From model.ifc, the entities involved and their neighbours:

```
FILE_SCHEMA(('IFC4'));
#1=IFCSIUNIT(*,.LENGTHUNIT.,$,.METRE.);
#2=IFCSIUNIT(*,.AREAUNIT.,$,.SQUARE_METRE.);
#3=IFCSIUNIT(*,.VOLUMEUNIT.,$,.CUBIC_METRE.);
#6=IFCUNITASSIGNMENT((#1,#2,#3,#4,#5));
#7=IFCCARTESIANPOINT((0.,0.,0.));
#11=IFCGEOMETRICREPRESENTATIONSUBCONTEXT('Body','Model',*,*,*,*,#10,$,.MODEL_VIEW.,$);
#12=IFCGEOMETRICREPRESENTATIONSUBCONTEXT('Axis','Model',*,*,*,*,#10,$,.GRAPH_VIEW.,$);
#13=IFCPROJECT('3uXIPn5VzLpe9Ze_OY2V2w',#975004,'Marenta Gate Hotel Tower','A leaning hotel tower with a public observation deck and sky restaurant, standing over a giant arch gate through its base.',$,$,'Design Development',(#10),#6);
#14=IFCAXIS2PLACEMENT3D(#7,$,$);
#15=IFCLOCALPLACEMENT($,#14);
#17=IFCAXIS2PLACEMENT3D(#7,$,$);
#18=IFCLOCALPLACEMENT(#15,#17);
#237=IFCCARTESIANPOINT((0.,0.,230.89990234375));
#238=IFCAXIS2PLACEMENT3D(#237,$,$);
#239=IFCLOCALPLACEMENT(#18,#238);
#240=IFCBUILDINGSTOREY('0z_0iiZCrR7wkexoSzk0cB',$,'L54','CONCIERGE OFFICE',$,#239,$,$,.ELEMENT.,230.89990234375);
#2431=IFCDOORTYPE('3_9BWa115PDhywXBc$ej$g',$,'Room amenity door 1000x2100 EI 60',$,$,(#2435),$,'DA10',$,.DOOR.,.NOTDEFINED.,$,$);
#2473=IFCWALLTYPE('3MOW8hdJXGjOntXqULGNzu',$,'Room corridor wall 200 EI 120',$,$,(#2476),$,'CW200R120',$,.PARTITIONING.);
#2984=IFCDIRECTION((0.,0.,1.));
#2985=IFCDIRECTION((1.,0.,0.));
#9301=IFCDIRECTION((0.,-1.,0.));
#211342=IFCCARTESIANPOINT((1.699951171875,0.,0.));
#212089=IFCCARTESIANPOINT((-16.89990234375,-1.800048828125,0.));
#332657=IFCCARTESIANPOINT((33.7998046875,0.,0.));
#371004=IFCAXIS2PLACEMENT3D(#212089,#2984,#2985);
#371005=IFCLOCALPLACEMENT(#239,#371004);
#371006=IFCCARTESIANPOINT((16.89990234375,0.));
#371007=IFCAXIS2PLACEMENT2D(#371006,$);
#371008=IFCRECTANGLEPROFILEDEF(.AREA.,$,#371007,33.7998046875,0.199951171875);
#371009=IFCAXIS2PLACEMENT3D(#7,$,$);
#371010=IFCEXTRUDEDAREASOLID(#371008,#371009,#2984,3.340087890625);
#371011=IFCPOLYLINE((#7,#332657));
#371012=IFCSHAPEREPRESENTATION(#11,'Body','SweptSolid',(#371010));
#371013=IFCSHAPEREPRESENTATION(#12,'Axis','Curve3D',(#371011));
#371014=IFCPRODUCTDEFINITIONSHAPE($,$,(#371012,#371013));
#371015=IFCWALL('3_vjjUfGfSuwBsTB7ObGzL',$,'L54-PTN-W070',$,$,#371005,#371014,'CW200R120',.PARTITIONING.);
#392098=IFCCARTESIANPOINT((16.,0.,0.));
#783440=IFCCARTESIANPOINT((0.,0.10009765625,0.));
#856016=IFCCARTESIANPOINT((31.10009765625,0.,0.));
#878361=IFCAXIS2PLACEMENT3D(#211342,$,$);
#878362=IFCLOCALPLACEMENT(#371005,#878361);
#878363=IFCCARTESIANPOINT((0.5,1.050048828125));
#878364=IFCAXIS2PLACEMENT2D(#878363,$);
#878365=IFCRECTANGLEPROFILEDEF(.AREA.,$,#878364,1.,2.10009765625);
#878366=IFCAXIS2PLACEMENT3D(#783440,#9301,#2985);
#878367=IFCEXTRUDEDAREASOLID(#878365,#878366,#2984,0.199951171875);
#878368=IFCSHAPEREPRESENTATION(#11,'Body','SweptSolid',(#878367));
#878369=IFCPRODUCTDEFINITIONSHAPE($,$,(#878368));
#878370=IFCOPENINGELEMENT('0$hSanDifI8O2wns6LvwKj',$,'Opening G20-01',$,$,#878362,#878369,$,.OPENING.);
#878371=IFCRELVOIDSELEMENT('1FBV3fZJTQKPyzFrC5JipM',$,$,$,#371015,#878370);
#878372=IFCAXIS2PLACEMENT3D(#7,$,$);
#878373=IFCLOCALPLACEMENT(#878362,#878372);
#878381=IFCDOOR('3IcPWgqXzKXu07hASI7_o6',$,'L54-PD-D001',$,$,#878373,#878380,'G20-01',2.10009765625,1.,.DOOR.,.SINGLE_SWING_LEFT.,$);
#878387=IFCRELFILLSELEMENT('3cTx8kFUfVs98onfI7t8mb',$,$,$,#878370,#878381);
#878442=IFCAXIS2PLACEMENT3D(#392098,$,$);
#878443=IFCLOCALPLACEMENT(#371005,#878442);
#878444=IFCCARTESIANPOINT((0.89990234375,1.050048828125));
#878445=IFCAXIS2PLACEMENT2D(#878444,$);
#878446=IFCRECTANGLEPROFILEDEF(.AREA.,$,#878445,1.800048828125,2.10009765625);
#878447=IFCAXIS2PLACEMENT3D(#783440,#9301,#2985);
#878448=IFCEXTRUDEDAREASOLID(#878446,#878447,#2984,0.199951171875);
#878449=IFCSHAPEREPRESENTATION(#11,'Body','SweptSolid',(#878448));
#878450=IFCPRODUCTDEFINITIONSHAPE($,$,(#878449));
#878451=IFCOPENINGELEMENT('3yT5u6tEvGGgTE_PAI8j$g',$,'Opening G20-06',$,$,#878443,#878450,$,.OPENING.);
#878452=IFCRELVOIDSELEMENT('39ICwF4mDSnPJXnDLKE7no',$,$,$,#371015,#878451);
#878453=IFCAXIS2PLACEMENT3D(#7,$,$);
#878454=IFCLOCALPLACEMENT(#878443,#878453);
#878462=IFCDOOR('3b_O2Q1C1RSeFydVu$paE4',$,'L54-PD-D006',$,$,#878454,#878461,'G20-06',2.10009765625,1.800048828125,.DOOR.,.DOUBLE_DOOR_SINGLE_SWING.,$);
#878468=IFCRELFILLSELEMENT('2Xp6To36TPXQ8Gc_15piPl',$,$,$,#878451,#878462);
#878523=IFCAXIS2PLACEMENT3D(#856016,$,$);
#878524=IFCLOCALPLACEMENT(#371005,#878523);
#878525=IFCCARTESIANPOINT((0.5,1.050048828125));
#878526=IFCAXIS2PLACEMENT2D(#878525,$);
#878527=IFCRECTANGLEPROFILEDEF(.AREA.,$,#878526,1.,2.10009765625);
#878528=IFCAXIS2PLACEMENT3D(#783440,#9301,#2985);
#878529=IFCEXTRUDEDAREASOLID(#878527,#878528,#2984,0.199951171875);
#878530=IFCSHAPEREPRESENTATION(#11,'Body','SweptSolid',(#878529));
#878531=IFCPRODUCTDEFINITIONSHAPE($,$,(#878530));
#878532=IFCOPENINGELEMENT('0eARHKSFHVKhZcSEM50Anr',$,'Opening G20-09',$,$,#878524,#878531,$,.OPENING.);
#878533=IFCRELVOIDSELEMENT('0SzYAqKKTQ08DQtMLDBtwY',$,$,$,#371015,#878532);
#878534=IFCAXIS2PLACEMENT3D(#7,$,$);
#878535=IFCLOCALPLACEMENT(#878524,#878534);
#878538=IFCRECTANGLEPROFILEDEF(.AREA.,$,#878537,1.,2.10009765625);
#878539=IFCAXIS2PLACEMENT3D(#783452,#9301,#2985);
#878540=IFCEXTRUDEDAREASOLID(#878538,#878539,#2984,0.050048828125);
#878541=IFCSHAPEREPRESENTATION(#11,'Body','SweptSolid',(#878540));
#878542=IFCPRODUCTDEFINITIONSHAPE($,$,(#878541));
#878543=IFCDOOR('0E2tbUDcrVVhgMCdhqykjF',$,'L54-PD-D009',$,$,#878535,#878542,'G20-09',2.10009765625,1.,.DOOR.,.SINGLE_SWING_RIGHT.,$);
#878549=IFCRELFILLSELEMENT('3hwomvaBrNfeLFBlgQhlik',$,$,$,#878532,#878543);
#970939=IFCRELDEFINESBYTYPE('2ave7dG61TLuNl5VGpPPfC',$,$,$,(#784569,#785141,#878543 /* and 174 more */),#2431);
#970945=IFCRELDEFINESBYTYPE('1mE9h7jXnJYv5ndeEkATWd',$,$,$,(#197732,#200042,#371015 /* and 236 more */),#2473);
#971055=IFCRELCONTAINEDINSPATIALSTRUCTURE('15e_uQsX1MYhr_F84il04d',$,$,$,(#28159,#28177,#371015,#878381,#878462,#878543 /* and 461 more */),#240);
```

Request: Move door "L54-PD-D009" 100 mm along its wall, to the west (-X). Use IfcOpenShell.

```python
import ifcopenshell
import ifcopenshell.api.geometry
import ifcopenshell.util.placement

model = ifcopenshell.open("model.ifc")

door = model.by_id(878543)
opening = door.FillsVoids[0].RelatingOpeningElement
wall = opening.VoidsElements[0].RelatingBuildingElement

wall_matrix = ifcopenshell.util.placement.get_local_placement(wall.ObjectPlacement)
shift = wall_matrix[:3, 0] * -0.1
before = ifcopenshell.util.placement.get_local_placement(door.ObjectPlacement)[:3, 3].copy()

# The door is placed relative to its opening, so it follows when the opening moves.
matrix = ifcopenshell.util.placement.get_local_placement(opening.ObjectPlacement)
matrix[:3, 3] += shift
ifcopenshell.api.geometry.edit_object_placement(
    model, product=opening, matrix=matrix, is_si=False, should_transform_children=True
)

after = ifcopenshell.util.placement.get_local_placement(door.ObjectPlacement)[:3, 3]
print("door moved by", (after - before).round(3) + 0.0)

model.write("model_edited.ifc")
```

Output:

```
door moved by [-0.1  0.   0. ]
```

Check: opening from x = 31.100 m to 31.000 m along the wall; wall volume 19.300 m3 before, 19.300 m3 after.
